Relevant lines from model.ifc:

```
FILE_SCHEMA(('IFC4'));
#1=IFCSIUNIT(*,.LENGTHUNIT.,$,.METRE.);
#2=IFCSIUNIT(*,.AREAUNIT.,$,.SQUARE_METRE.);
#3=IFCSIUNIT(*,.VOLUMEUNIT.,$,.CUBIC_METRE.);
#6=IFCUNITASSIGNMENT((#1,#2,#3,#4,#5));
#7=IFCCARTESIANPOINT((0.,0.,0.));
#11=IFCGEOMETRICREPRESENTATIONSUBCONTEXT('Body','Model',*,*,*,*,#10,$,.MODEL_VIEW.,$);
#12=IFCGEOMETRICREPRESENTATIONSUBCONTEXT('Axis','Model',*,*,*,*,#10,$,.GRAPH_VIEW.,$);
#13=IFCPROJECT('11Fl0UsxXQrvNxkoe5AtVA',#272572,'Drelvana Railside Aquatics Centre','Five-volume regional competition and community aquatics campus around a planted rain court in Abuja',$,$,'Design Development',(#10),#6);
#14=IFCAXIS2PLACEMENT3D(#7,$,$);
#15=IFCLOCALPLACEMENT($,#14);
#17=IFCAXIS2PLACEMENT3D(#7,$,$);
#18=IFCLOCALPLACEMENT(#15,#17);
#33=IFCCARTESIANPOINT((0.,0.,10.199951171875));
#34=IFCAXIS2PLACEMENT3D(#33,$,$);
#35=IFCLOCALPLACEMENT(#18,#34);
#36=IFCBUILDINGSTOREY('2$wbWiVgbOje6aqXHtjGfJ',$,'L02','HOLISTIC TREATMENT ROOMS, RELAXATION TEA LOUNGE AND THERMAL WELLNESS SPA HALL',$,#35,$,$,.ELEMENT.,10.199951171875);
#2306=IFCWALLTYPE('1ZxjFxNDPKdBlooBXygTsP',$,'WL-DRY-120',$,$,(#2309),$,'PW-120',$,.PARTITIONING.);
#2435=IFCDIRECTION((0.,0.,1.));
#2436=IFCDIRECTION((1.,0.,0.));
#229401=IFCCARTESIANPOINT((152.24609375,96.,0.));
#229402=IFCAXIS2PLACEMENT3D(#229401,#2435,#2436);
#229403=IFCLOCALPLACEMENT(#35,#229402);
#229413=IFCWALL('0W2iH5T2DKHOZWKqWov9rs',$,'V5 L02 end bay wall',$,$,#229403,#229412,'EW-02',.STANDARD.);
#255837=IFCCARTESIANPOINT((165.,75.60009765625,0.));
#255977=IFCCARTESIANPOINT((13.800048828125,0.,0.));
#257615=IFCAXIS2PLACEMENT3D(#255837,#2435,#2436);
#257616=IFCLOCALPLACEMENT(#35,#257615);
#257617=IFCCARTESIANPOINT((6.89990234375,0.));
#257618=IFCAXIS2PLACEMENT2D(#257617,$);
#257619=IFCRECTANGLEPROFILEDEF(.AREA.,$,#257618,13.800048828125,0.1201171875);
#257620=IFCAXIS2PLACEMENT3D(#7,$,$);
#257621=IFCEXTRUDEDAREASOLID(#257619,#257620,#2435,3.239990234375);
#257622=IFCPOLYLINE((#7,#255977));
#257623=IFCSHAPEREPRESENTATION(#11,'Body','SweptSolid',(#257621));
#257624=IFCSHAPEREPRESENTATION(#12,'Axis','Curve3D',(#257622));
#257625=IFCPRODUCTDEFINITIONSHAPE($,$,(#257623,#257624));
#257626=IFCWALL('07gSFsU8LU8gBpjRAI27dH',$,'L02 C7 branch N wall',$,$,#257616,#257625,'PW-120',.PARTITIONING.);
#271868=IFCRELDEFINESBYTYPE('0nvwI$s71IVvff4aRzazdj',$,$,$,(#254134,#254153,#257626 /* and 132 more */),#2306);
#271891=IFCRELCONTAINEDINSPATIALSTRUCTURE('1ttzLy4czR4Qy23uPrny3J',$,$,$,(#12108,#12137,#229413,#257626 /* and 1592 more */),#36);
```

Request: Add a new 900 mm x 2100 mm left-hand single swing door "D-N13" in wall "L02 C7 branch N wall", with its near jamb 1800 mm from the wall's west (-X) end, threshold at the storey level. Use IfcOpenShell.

```python
import numpy as np
import ifcopenshell
import ifcopenshell.api.feature
import ifcopenshell.api.geometry
import ifcopenshell.api.root
import ifcopenshell.api.spatial
import ifcopenshell.geom
import ifcopenshell.util.element
import ifcopenshell.util.placement
import ifcopenshell.util.representation
import ifcopenshell.util.shape
import ifcopenshell.util.unit

model = ifcopenshell.open("model.ifc")
unit_scale = ifcopenshell.util.unit.calculate_unit_scale(model)
settings = ifcopenshell.geom.settings()


def volume(element):
    """Net volume in cubic metres, openings subtracted."""
    shape = ifcopenshell.geom.create_shape(settings, element)
    return ifcopenshell.util.shape.get_volume(shape.geometry)


wall = model.by_guid("07gSFsU8LU8gBpjRAI27dH")
storey = ifcopenshell.util.element.get_container(wall, ifc_class="IfcBuildingStorey")
context = ifcopenshell.util.representation.get_context(model, "Model", "Body", "MODEL_VIEW")
before = volume(wall)

width, height, from_end, sill = 0.9, 2.1, 1.8, 0.0  # metres

# The wall runs along its own X axis, and the end named is its -X end.
wall_shape = ifcopenshell.geom.create_shape(settings, wall)
x, y, z = ifcopenshell.util.shape.get_vertices(wall_shape.geometry).T
start = x.min() + from_end
face, thickness = float(y.min()), float(y.max() - y.min())
wall_matrix = ifcopenshell.util.placement.get_local_placement(wall.ObjectPlacement)
level = ifcopenshell.util.placement.get_local_placement(storey.ObjectPlacement)[2, 3]


def in_wall(x, y):
    """Placement at x, y metres in the wall's axes, at sill height."""
    matrix = wall_matrix.copy()
    matrix[:, 3] = wall_matrix @ np.array([x / unit_scale, y / unit_scale, 0.0, 1.0])
    matrix[2, 3] = level + sill / unit_scale
    return matrix


# Opening: a box that overshoots both wall faces by 50 mm.
opening = ifcopenshell.api.root.create_entity(model, ifc_class="IfcOpeningElement", predefined_type="OPENING")
box = ifcopenshell.api.geometry.add_wall_representation(
    model, context=context, length=width, height=height, thickness=thickness + 0.1
)
ifcopenshell.api.geometry.assign_representation(model, product=opening, representation=box)
ifcopenshell.api.geometry.edit_object_placement(model, product=opening, matrix=in_wall(start, face - 0.05), is_si=False)
ifcopenshell.api.feature.add_feature(model, feature=opening, element=wall)

door = ifcopenshell.api.root.create_entity(model, ifc_class="IfcDoor", name="D-N13", predefined_type="DOOR")
door.OverallWidth, door.OverallHeight = width / unit_scale, height / unit_scale
door.OperationType = "SINGLE_SWING_LEFT"
body = ifcopenshell.api.geometry.add_door_representation(
    model,
    context=context,
    overall_width=door.OverallWidth,
    overall_height=door.OverallHeight,
    operation_type="SINGLE_SWING_LEFT",
    lining_properties={"LiningDepth": thickness / unit_scale, "ThresholdDepth": thickness / unit_scale},
)
ifcopenshell.api.geometry.assign_representation(model, product=door, representation=body)
ifcopenshell.api.spatial.assign_container(model, products=[door], relating_structure=storey)
ifcopenshell.api.feature.add_filling(model, opening=opening, element=door)

# The lining spans the wall, so the door starts at the wall face.
ifcopenshell.api.geometry.edit_object_placement(model, product=door, matrix=in_wall(start, face), is_si=False)

after = volume(wall)

print(f"wall volume {before:.3f} -> {after:.3f} m3")

model.write("model_edited.ifc")
```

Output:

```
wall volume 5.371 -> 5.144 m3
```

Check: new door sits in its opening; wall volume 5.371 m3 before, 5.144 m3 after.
